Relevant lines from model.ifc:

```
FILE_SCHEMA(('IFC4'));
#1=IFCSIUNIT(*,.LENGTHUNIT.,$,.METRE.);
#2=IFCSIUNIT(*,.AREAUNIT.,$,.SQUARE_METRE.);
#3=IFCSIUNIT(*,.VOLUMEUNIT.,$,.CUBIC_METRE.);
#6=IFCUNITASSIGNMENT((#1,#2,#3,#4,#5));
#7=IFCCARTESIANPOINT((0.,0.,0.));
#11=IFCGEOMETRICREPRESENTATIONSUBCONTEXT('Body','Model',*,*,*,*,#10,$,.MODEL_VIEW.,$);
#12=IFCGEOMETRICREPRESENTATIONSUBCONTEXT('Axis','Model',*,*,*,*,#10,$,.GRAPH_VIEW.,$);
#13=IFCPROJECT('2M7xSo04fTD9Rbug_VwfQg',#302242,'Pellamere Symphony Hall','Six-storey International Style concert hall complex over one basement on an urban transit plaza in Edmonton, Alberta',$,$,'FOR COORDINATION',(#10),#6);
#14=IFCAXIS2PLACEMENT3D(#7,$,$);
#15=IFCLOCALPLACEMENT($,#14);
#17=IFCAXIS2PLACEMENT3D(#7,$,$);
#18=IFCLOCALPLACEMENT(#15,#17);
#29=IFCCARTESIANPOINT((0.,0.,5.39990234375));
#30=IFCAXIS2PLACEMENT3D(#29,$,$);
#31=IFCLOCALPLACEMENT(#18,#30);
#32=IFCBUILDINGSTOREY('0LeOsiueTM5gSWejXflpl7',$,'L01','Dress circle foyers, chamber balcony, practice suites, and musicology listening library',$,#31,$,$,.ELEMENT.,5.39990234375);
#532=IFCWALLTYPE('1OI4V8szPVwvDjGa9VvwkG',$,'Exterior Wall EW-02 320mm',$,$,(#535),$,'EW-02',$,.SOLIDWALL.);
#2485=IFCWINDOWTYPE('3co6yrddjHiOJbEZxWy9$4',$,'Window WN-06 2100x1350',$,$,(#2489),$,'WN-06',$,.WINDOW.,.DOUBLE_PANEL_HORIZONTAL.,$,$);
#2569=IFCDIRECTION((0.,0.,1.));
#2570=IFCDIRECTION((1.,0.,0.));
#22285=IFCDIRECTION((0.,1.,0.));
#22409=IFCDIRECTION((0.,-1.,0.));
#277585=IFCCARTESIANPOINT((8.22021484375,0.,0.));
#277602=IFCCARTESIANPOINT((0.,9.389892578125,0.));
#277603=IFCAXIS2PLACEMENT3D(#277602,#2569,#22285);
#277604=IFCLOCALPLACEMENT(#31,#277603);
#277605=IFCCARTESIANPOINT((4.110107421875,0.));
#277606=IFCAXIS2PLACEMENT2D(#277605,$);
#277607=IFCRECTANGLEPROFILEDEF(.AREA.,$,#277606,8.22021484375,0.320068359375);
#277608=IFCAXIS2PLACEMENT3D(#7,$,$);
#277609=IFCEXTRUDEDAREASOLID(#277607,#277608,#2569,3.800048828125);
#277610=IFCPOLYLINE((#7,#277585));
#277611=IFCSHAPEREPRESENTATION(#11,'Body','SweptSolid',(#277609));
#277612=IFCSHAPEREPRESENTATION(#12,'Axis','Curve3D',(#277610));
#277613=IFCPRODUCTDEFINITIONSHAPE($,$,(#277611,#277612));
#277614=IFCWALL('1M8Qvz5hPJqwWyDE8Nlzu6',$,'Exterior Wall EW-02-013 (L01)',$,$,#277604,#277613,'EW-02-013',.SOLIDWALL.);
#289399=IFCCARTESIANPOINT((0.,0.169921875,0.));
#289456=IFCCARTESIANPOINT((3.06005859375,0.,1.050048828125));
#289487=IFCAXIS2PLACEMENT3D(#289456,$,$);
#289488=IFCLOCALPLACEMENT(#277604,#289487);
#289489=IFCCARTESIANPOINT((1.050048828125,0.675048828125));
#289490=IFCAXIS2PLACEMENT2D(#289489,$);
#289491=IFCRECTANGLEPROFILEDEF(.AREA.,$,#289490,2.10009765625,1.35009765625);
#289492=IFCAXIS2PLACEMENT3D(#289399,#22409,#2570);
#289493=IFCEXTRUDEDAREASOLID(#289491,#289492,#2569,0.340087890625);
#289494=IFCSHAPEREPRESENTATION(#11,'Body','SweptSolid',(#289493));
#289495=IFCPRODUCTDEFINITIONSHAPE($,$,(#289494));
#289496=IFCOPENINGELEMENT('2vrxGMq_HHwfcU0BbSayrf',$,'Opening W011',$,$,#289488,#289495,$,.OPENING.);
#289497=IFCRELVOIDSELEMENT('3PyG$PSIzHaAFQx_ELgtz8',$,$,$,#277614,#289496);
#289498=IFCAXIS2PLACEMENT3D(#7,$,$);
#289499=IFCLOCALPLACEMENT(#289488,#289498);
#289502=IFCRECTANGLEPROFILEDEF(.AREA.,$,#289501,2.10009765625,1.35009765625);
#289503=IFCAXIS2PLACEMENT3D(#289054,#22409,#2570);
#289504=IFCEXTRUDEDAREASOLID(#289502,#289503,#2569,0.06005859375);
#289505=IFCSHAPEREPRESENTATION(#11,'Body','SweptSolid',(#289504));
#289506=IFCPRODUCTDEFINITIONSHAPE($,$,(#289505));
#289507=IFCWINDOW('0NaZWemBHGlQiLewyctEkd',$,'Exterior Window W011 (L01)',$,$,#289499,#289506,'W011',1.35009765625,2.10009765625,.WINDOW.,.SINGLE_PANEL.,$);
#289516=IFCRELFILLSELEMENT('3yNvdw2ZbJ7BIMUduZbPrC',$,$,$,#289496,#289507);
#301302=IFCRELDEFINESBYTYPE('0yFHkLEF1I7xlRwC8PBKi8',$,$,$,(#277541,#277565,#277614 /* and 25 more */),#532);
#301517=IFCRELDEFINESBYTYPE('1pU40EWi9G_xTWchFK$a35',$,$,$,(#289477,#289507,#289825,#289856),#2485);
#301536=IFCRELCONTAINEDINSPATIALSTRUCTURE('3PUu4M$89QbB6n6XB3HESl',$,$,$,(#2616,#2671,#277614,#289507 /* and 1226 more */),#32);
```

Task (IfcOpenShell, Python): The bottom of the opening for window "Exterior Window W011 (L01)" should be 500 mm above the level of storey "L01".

```python
import numpy as np
import ifcopenshell
import ifcopenshell.api.geometry
import ifcopenshell.geom
import ifcopenshell.util.element
import ifcopenshell.util.placement
import ifcopenshell.util.shape
import ifcopenshell.util.unit

model = ifcopenshell.open("model.ifc")
unit_scale = ifcopenshell.util.unit.calculate_unit_scale(model)

window = model.by_guid("0NaZWemBHGlQiLewyctEkd")
opening = window.FillsVoids[0].RelatingOpeningElement
storey = ifcopenshell.util.element.get_container(window, ifc_class="IfcBuildingStorey")
level = ifcopenshell.util.placement.get_local_placement(storey.ObjectPlacement)[2, 3]

# The opening's origin need not be at the sill, so measure its lowest point.
shape = ifcopenshell.geom.create_shape(ifcopenshell.geom.settings(), opening)
bottom = ifcopenshell.util.shape.get_shape_bottom_elevation(shape, shape.geometry) / unit_scale
dz = level + 0.5 - bottom

shift = np.array([0.0, 0.0, dz])
# The window is placed relative to its opening, so it follows when the opening moves.
matrix = ifcopenshell.util.placement.get_local_placement(opening.ObjectPlacement)
matrix[:3, 3] += shift
ifcopenshell.api.geometry.edit_object_placement(
    model, product=opening, matrix=matrix, is_si=False, should_transform_children=True
)

print(f"moved by {dz * unit_scale:+.3f} m")

model.write("model_v2.ifc")
```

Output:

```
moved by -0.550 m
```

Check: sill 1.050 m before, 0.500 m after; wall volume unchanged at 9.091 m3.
